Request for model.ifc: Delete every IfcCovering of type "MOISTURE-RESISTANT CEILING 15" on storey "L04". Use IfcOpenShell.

First a look at what the model holds.

```python
import ifcopenshell
import ifcopenshell.util.element

model = ifcopenshell.open("model.ifc")
print(model.schema)
storey = next(s for s in model.by_type("IfcBuildingStorey") if s.Name == "L04")
coverings = [e for e in ifcopenshell.util.element.get_decomposition(storey) if e.is_a("IfcCovering")]
seen = {}
for e in coverings:
    element_type = ifcopenshell.util.element.get_type(e)
    name = element_type.Name if element_type not in (None, e) else None
    seen[name] = seen.get(name, 0) + 1
for name, count in sorted(seen.items(), key=str):
    print(count, "x", name)
```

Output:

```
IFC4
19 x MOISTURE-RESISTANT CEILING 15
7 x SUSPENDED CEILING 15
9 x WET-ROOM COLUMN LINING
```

```python
import ifcopenshell
import ifcopenshell.api.root
import ifcopenshell.util.element

model = ifcopenshell.open("model.ifc")

storey = next(s for s in model.by_type("IfcBuildingStorey") if s.Name == "L04")
coverings = [e for e in ifcopenshell.util.element.get_decomposition(storey) if e.is_a("IfcCovering")]
targets = [e for e in coverings if (t := ifcopenshell.util.element.get_type(e)) not in (None, e) and t.Name == "MOISTURE-RESISTANT CEILING 15"]

for e in targets:
    ifcopenshell.api.root.remove_product(model, product=e)
print(len(targets), "removed")

model.write("model_edited.ifc")
```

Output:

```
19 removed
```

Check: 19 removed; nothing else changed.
